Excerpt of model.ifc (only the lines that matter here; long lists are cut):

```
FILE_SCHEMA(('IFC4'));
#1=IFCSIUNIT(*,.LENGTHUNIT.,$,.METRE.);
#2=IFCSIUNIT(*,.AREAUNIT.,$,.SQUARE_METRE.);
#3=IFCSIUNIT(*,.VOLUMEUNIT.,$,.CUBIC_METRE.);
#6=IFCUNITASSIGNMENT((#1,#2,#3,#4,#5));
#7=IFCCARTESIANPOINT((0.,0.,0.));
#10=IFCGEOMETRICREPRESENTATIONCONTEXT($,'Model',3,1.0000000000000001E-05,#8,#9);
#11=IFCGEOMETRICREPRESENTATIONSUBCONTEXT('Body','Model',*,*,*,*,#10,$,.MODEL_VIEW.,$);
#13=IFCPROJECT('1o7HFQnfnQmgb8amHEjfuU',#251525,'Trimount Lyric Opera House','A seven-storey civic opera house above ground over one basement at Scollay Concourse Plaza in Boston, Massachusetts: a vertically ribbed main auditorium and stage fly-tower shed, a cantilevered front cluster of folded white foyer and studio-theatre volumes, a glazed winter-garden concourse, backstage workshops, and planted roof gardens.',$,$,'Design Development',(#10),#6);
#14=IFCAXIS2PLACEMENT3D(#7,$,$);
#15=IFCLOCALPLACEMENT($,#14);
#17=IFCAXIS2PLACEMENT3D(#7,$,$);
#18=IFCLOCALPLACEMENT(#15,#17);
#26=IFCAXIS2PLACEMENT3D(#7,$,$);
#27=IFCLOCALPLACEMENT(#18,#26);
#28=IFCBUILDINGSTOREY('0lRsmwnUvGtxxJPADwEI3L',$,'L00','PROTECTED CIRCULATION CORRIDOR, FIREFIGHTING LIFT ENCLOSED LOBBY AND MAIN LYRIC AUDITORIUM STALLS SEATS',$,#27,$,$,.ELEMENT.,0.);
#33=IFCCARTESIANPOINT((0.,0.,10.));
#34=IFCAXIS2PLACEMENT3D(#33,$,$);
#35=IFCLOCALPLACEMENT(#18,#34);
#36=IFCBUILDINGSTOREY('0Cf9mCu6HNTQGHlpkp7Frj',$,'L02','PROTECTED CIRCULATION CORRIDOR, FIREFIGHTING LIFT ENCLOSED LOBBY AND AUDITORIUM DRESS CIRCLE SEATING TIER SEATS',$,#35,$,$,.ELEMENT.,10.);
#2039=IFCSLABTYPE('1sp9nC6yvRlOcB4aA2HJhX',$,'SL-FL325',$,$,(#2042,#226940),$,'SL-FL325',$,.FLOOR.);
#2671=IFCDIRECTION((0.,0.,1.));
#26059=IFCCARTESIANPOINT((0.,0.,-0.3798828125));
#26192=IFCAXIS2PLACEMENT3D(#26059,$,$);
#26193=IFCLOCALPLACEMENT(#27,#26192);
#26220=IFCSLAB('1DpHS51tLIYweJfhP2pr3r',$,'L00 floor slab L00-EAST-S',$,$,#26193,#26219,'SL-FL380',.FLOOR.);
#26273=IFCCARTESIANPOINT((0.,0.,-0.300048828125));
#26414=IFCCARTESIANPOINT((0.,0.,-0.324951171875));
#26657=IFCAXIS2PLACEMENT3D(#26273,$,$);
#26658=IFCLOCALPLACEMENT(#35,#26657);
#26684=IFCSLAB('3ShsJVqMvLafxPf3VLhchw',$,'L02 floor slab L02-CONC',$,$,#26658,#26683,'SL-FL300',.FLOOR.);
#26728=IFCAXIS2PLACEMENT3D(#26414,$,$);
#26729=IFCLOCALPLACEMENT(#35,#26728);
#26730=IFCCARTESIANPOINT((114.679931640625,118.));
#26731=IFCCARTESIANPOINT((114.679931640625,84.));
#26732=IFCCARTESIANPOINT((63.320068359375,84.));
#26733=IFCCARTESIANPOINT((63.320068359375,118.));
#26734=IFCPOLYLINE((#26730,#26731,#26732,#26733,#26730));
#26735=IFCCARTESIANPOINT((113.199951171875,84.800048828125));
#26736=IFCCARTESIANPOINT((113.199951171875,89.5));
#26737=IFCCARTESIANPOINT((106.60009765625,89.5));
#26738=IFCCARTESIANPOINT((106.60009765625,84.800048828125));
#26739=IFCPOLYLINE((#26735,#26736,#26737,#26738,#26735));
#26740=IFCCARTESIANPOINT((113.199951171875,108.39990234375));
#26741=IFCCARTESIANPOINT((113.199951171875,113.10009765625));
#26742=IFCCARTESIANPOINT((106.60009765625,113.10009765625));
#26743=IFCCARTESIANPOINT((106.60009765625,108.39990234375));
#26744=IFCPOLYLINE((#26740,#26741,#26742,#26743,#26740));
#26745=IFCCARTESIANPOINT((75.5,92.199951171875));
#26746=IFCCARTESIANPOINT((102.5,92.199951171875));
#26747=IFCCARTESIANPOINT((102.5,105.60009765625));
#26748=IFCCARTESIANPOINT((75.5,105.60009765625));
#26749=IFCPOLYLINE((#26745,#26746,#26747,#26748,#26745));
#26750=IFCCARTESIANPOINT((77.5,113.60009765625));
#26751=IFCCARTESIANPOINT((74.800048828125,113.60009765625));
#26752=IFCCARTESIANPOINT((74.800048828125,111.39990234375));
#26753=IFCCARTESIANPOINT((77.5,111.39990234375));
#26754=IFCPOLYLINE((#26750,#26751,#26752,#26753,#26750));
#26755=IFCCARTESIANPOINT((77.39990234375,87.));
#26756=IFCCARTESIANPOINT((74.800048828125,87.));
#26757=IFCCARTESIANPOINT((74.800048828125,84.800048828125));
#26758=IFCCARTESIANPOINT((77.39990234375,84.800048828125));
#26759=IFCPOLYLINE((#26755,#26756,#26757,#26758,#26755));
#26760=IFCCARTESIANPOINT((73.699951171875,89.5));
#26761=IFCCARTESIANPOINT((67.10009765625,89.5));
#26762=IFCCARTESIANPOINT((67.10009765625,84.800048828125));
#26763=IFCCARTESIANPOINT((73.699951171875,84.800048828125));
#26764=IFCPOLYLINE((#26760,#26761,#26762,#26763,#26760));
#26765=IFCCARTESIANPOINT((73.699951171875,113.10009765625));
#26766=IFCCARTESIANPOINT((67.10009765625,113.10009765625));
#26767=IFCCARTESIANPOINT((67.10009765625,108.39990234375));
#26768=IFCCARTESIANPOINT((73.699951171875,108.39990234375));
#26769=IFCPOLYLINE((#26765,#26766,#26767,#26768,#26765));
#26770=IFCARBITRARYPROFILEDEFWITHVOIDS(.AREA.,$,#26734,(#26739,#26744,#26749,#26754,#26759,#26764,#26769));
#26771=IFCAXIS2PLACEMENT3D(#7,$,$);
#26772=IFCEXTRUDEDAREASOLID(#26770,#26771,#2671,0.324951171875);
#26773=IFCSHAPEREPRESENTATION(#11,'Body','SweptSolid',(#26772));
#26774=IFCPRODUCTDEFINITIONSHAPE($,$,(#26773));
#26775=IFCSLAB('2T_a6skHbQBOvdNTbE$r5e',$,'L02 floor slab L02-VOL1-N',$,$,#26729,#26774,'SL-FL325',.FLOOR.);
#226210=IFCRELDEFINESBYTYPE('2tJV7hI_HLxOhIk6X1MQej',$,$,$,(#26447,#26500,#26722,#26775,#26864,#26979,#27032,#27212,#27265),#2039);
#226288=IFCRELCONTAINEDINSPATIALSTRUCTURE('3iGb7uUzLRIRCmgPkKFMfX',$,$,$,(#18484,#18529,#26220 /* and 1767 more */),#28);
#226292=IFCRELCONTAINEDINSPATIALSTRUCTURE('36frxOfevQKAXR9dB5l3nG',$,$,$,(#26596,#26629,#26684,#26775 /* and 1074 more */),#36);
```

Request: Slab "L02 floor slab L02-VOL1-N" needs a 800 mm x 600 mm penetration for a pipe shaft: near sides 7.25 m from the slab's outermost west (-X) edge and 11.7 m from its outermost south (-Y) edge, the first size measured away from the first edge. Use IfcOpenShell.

```python
import numpy as np
import ifcopenshell
import ifcopenshell.api.feature
import ifcopenshell.api.geometry
import ifcopenshell.api.root
import ifcopenshell.geom
import ifcopenshell.util.placement
import ifcopenshell.util.representation
import ifcopenshell.util.shape
import ifcopenshell.util.unit

model = ifcopenshell.open("model.ifc")
unit_scale = ifcopenshell.util.unit.calculate_unit_scale(model)
settings = ifcopenshell.geom.settings()


def volume(element):
    """Net volume in cubic metres, openings subtracted."""
    shape = ifcopenshell.geom.create_shape(settings, element)
    return ifcopenshell.util.shape.get_volume(shape.geometry)


slab = model.by_id(26775)
before = volume(slab)

# Extent in the slab's own axes, in metres. The edges named are its -X and -Y sides.
slab_shape = ifcopenshell.geom.create_shape(settings, slab)
vertices = ifcopenshell.util.shape.get_vertices(slab_shape.geometry)
x_min, y_min, bottom = vertices.min(axis=0)
top = vertices[:, 2].max()

opening = ifcopenshell.api.root.create_entity(model, ifc_class="IfcOpeningElement", name="Pipe shaft opening", predefined_type="OPENING")
context = ifcopenshell.util.representation.get_context(model, "Model", "Body", "MODEL_VIEW")
width, depth = 0.8, 0.6
outline = [(0.0, 0.0), (width, 0.0), (width, depth), (0.0, depth), (0.0, 0.0)]
# Overshoot both faces by 50 mm so the cut is clean.
shape = ifcopenshell.api.geometry.add_slab_representation(
    model, context=context, depth=top - bottom + 0.1, polyline=outline
)
ifcopenshell.api.geometry.assign_representation(model, product=opening, representation=shape)

matrix = ifcopenshell.util.placement.get_local_placement(slab.ObjectPlacement)
matrix[:, 3] = matrix @ np.append(np.array([x_min + 7.25, y_min + 11.7, bottom - 0.05]) / unit_scale, 1.0)
ifcopenshell.api.geometry.edit_object_placement(model, product=opening, matrix=matrix, is_si=False)
ifcopenshell.api.feature.add_feature(model, feature=opening, element=slab)

after = volume(slab)

print(f"slab volume {before:.3f} -> {after:.3f} m3")

model.write("model_updated.ifc")
```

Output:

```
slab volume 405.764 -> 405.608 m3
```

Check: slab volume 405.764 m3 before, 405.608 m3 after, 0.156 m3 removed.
